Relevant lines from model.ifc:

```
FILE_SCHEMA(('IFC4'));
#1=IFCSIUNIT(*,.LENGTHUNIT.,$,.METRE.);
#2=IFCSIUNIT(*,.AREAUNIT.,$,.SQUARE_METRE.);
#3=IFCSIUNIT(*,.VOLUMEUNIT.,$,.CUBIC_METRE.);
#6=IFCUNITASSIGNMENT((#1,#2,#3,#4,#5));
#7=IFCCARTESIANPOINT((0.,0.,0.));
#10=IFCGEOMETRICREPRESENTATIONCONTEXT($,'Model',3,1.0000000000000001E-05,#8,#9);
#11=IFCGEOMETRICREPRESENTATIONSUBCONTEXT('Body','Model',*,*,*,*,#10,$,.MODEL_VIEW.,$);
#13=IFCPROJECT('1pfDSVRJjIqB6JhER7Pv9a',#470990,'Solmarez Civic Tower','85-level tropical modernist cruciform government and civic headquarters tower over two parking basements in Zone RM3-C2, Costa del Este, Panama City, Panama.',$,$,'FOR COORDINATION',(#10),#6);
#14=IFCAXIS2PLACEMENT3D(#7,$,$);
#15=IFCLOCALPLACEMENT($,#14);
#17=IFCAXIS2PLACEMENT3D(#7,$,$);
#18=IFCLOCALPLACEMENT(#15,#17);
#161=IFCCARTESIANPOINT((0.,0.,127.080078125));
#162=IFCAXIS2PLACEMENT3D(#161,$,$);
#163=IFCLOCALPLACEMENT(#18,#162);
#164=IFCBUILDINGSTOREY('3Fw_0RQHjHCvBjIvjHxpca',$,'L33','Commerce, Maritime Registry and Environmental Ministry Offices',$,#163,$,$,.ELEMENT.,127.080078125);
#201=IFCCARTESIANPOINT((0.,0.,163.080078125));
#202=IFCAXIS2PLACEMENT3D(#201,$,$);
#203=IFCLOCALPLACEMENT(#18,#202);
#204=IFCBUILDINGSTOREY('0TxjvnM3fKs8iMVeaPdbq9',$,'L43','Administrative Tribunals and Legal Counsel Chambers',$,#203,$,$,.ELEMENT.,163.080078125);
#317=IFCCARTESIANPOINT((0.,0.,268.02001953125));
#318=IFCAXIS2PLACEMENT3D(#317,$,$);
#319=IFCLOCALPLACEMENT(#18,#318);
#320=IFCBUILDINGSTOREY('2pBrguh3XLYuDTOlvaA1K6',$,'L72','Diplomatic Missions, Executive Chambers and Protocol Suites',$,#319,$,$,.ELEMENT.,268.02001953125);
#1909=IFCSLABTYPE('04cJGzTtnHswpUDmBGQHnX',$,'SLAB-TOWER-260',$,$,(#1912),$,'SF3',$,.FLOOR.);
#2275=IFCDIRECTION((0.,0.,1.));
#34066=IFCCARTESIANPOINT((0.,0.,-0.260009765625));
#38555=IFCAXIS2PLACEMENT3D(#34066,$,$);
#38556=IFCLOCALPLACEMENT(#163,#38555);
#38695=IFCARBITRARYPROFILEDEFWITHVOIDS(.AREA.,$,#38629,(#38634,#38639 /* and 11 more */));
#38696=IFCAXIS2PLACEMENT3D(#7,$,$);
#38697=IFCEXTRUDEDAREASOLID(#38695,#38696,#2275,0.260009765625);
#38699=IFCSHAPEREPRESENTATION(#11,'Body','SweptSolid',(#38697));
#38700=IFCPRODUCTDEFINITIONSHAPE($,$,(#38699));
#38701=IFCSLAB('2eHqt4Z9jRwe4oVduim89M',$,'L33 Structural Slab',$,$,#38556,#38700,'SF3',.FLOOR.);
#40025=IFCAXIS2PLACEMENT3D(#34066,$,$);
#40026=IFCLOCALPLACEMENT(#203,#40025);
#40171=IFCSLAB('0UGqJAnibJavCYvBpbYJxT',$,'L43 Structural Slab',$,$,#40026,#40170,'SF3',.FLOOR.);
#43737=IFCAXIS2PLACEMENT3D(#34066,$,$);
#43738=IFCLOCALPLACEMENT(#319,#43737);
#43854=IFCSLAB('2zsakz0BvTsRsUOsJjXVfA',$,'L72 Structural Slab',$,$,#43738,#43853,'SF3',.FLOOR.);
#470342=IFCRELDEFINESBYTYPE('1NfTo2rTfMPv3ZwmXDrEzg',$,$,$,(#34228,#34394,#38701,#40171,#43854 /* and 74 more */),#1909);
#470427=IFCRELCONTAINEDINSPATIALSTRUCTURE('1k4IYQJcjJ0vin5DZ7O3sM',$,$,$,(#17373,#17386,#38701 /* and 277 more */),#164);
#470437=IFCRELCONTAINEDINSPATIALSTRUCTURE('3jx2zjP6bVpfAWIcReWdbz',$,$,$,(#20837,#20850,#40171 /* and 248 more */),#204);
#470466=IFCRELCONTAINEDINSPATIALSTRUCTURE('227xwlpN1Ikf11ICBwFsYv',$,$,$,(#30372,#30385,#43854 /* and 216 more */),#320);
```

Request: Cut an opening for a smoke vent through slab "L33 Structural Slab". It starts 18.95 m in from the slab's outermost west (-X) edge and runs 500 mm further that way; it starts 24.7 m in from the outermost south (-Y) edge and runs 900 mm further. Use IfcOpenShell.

```python
import numpy as np
import ifcopenshell
import ifcopenshell.api.feature
import ifcopenshell.api.geometry
import ifcopenshell.api.root
import ifcopenshell.geom
import ifcopenshell.util.placement
import ifcopenshell.util.representation
import ifcopenshell.util.shape
import ifcopenshell.util.unit

model = ifcopenshell.open("model.ifc")
unit_scale = ifcopenshell.util.unit.calculate_unit_scale(model)
settings = ifcopenshell.geom.settings()


def volume(element):
    """Net volume in cubic metres, openings subtracted."""
    shape = ifcopenshell.geom.create_shape(settings, element)
    return ifcopenshell.util.shape.get_volume(shape.geometry)


slab = model.by_id(38701)
before = volume(slab)

# Extent in the slab's own axes, in metres. The edges named are its -X and -Y sides.
slab_shape = ifcopenshell.geom.create_shape(settings, slab)
vertices = ifcopenshell.util.shape.get_vertices(slab_shape.geometry)
x_min, y_min, bottom = vertices.min(axis=0)
top = vertices[:, 2].max()

opening = ifcopenshell.api.root.create_entity(model, ifc_class="IfcOpeningElement", name="Smoke vent opening", predefined_type="OPENING")
context = ifcopenshell.util.representation.get_context(model, "Model", "Body", "MODEL_VIEW")
width, depth = 0.5, 0.9
outline = [(0.0, 0.0), (width, 0.0), (width, depth), (0.0, depth), (0.0, 0.0)]
# Overshoot both faces by 50 mm so the cut is clean.
shape = ifcopenshell.api.geometry.add_slab_representation(
    model, context=context, depth=top - bottom + 0.1, polyline=outline
)
ifcopenshell.api.geometry.assign_representation(model, product=opening, representation=shape)

matrix = ifcopenshell.util.placement.get_local_placement(slab.ObjectPlacement)
matrix[:, 3] = matrix @ np.append(np.array([x_min + 18.95, y_min + 24.7, bottom - 0.05]) / unit_scale, 1.0)
ifcopenshell.api.geometry.edit_object_placement(model, product=opening, matrix=matrix, is_si=False)
ifcopenshell.api.feature.add_feature(model, feature=opening, element=slab)

after = volume(slab)

print(f"slab volume {before:.3f} -> {after:.3f} m3")

model.write("model_rev.ifc")
```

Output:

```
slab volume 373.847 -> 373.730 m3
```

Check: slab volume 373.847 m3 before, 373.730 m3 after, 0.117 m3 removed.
